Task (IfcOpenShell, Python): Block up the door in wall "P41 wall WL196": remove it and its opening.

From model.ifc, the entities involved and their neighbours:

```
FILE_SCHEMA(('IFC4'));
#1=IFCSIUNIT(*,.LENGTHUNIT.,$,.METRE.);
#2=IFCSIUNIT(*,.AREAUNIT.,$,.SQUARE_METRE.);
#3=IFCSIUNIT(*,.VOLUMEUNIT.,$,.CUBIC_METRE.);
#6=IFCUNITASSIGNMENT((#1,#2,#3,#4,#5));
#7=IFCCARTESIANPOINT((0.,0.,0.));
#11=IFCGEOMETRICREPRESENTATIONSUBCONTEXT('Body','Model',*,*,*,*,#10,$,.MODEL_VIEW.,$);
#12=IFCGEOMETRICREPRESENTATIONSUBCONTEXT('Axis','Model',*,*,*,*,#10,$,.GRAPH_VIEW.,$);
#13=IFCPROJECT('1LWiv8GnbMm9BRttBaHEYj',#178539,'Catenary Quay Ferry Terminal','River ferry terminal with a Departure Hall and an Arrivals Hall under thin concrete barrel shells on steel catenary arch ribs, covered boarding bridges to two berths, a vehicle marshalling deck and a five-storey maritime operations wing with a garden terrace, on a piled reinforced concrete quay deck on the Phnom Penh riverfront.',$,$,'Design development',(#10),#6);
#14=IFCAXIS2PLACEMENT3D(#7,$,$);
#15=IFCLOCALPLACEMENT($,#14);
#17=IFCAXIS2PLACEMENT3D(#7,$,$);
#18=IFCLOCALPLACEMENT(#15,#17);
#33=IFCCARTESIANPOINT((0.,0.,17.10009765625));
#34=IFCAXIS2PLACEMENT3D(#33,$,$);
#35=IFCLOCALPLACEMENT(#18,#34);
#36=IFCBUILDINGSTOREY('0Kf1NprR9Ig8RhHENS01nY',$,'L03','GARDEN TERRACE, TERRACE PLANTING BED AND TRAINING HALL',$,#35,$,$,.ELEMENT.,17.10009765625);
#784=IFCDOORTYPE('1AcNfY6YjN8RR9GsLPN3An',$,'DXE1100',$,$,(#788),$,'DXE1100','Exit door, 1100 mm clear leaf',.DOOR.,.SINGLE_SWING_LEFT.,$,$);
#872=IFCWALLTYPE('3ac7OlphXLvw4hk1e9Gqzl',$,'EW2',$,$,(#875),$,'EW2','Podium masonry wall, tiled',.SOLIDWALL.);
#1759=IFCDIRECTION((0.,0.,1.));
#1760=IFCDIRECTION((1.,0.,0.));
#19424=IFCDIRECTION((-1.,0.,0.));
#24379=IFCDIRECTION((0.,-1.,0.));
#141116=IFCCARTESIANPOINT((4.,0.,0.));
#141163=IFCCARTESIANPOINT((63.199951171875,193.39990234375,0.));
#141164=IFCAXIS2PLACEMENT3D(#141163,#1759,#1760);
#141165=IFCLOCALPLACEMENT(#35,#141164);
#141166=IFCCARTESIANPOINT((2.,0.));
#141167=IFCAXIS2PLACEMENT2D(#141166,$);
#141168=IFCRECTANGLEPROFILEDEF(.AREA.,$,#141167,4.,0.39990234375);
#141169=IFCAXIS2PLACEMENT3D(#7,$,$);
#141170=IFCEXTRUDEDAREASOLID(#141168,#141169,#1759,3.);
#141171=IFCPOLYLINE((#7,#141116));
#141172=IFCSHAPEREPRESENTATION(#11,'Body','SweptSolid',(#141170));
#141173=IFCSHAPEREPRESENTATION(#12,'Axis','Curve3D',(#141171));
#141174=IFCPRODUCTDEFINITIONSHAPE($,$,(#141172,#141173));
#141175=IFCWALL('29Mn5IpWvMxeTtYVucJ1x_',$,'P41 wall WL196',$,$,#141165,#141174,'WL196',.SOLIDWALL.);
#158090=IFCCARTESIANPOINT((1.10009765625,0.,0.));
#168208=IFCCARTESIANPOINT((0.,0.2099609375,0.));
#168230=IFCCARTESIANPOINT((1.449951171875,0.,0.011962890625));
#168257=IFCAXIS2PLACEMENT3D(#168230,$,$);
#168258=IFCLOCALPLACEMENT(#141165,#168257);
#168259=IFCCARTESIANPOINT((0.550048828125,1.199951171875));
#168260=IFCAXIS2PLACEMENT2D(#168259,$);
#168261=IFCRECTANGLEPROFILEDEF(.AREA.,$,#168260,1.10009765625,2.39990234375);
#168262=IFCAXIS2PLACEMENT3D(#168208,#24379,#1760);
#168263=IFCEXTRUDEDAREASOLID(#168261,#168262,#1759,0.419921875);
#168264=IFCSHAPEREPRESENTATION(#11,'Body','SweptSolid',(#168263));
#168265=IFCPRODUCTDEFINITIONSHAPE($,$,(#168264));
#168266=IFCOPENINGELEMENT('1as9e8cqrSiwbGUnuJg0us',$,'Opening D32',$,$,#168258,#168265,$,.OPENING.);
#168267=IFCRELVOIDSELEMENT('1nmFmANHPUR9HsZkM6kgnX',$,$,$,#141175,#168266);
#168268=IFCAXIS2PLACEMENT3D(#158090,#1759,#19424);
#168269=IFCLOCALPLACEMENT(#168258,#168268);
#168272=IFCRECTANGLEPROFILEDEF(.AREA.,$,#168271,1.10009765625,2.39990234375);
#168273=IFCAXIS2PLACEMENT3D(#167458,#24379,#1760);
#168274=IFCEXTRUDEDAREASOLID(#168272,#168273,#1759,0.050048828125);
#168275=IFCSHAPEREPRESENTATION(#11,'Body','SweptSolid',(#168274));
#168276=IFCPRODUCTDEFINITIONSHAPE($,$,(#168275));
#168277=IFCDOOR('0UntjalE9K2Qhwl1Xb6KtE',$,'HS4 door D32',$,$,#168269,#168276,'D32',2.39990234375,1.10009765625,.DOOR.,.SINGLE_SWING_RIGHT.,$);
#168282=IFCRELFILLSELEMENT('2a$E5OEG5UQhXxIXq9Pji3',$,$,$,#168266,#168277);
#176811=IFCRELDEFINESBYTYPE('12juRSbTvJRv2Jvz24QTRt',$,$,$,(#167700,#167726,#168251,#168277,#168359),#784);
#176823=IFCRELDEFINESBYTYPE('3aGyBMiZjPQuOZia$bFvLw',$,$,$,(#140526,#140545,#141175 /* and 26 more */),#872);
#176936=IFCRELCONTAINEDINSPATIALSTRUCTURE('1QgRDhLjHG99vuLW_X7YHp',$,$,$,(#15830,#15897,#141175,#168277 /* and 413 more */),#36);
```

```python
import ifcopenshell
import ifcopenshell.api.feature
import ifcopenshell.api.root
import ifcopenshell.geom
import ifcopenshell.util.shape

model = ifcopenshell.open("model.ifc")
settings = ifcopenshell.geom.settings()


def volume(element):
    """Net volume in cubic metres, openings subtracted."""
    shape = ifcopenshell.geom.create_shape(settings, element)
    return ifcopenshell.util.shape.get_volume(shape.geometry)


door = model.by_guid("0UntjalE9K2Qhwl1Xb6KtE")
opening = door.FillsVoids[0].RelatingOpeningElement
wall = opening.VoidsElements[0].RelatingBuildingElement
before = volume(wall)

ifcopenshell.api.root.remove_product(model, product=door)
ifcopenshell.api.feature.remove_feature(model, feature=opening)

after = volume(wall)

print(f"wall volume {before:.3f} -> {after:.3f} m3")

model.write("model_updated.ifc")
```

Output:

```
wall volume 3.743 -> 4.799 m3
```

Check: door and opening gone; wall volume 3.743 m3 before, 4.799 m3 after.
